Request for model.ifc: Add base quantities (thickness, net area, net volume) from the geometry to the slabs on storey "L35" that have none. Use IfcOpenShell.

First a look at what the model holds.

```python
import ifcopenshell
import ifcopenshell.util.element
import ifcopenshell.util.unit

model = ifcopenshell.open("model.ifc")
print(model.schema)
for unit_type in ("LENGTHUNIT", "AREAUNIT", "VOLUMEUNIT"):
    print(unit_type, ifcopenshell.util.unit.calculate_unit_scale(model, unit_type))
storey = next(s for s in model.by_type("IfcBuildingStorey") if s.Name == "L35")
slabs = [e for e in ifcopenshell.util.element.get_decomposition(storey) if e.is_a("IfcSlab")]
for e in sorted(slabs, key=lambda e: e.id()):
    print(e.id(), e.is_a(), e.Name, list(ifcopenshell.util.element.get_psets(e, qtos_only=True)), sep=" | ")
```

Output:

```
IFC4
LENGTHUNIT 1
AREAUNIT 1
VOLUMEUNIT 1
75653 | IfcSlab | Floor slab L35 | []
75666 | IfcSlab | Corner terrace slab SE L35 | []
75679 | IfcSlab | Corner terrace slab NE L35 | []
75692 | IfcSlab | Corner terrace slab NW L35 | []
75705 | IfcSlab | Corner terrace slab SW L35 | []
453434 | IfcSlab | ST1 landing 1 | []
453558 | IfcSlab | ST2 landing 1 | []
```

```python
import ifcopenshell
import ifcopenshell.api.pset
import ifcopenshell.geom
import ifcopenshell.util.element
import ifcopenshell.util.shape
import ifcopenshell.util.unit

model = ifcopenshell.open("model.ifc")
unit_scale = ifcopenshell.util.unit.calculate_unit_scale(model)
area_scale = ifcopenshell.util.unit.calculate_unit_scale(model, "AREAUNIT")
volume_scale = ifcopenshell.util.unit.calculate_unit_scale(model, "VOLUMEUNIT")
settings = ifcopenshell.geom.settings()

storey = next(s for s in model.by_type("IfcBuildingStorey") if s.Name == "L35")
slabs = [e for e in ifcopenshell.util.element.get_decomposition(storey) if e.is_a("IfcSlab")]

for e in sorted(slabs, key=lambda e: e.id()):
    if ifcopenshell.util.element.get_psets(e, qtos_only=True, should_inherit=False):
        continue
    # Geometry comes back in metres, in the element's own axes.
    shape = ifcopenshell.geom.create_shape(settings, e)
    values = {
        "Width": ifcopenshell.util.shape.get_z(shape.geometry) / unit_scale,
        "NetArea": ifcopenshell.util.shape.get_footprint_area(shape.geometry) / area_scale,
        "NetVolume": ifcopenshell.util.shape.get_volume(shape.geometry) / volume_scale,
    }
    qto = ifcopenshell.api.pset.add_qto(model, product=e, name="Qto_SlabBaseQuantities")
    ifcopenshell.api.pset.edit_qto(model, qto=qto, properties=values)
    print(e.id(), {k: round(v, 3) for k, v in values.items()})

model.write("model_rev.ifc")
```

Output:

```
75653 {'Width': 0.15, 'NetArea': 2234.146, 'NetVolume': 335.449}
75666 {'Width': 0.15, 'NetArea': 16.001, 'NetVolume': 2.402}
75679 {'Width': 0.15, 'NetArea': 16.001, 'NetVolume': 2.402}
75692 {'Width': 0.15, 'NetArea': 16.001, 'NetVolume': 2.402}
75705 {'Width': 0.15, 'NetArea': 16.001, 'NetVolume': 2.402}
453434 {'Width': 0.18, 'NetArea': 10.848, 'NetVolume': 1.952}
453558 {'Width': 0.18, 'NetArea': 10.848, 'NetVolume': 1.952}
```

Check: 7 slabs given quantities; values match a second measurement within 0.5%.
